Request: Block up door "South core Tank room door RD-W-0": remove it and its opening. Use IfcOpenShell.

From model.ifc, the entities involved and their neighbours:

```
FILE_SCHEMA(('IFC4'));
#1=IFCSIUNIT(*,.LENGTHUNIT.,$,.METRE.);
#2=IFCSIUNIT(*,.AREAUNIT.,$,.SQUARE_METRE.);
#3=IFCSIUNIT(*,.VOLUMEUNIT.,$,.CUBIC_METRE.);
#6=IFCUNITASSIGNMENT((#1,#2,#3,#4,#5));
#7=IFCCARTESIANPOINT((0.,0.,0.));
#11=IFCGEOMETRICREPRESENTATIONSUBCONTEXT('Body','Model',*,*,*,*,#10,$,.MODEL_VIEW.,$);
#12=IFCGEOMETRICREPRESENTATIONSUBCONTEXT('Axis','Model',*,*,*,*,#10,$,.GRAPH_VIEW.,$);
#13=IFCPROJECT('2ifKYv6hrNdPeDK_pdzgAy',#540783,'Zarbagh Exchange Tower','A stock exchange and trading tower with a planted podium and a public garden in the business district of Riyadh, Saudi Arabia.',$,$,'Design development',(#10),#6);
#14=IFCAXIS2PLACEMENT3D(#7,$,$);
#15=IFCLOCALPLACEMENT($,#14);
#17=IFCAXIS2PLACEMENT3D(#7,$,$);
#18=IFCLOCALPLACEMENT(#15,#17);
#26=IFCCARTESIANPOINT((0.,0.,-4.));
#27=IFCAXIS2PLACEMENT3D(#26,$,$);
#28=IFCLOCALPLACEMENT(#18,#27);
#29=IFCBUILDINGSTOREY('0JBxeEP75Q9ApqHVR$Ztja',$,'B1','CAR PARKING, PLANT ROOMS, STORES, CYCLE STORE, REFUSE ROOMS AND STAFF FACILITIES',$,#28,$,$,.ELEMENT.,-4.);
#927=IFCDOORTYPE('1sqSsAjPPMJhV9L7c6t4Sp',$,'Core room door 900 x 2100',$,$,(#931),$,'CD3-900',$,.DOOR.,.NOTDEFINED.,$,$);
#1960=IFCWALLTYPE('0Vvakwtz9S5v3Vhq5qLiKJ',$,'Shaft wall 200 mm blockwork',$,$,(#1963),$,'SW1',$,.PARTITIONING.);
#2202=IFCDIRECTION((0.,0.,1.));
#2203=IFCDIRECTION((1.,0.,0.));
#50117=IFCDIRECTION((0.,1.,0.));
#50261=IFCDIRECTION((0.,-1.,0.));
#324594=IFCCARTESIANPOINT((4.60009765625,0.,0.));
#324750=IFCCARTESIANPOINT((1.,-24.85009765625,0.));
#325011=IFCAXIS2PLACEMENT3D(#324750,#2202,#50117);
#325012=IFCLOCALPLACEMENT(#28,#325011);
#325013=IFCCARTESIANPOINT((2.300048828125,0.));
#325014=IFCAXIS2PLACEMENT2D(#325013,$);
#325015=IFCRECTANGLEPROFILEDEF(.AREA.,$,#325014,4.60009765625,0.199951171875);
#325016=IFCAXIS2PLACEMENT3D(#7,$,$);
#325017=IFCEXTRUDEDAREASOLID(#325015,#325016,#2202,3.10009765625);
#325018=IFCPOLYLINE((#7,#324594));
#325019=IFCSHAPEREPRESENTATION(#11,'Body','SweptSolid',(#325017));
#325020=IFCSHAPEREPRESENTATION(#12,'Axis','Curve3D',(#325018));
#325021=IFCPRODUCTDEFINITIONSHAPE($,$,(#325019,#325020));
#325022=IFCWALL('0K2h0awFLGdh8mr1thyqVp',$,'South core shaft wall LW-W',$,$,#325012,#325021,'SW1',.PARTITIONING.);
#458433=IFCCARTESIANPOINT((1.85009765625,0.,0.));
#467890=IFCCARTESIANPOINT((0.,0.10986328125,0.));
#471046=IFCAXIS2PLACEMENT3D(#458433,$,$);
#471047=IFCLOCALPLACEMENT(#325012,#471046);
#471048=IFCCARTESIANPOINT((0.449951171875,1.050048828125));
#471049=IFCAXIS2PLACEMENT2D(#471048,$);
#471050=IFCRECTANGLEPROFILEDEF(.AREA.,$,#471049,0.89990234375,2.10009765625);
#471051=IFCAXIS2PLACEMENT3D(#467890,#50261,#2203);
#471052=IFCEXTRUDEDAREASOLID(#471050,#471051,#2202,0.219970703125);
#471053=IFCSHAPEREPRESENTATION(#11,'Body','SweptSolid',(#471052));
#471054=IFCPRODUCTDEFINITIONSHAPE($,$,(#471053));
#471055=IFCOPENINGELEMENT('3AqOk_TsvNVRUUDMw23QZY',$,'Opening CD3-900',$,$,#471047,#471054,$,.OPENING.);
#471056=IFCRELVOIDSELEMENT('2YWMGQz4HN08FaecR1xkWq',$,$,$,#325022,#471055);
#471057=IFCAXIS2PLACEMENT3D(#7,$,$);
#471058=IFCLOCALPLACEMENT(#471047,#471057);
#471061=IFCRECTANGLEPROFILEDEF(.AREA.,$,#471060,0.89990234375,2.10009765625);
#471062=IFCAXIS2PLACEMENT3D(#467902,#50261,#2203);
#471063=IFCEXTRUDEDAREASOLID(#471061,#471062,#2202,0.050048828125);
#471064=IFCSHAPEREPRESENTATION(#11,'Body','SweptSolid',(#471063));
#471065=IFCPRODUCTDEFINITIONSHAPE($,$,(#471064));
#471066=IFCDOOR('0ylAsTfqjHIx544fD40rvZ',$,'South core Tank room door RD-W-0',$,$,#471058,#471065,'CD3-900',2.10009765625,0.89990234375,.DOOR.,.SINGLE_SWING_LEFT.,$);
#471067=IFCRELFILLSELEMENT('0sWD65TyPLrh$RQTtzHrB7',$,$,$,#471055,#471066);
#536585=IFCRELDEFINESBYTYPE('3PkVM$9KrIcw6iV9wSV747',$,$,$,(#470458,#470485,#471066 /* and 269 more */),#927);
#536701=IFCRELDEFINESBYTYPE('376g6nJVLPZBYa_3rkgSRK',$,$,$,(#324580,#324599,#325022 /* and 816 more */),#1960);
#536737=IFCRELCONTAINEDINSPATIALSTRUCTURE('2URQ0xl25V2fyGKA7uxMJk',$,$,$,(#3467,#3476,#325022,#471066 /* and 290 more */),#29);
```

```python
import ifcopenshell
import ifcopenshell.api.feature
import ifcopenshell.api.root
import ifcopenshell.geom
import ifcopenshell.util.shape

model = ifcopenshell.open("model.ifc")
settings = ifcopenshell.geom.settings()


def volume(element):
    """Net volume in cubic metres, openings subtracted."""
    shape = ifcopenshell.geom.create_shape(settings, element)
    return ifcopenshell.util.shape.get_volume(shape.geometry)


door = model.by_guid("0ylAsTfqjHIx544fD40rvZ")
opening = door.FillsVoids[0].RelatingOpeningElement
wall = opening.VoidsElements[0].RelatingBuildingElement
before = volume(wall)

ifcopenshell.api.root.remove_product(model, product=door)
ifcopenshell.api.feature.remove_feature(model, feature=opening)

after = volume(wall)

print(f"wall volume {before:.3f} -> {after:.3f} m3")

model.write("model_updated.ifc")
```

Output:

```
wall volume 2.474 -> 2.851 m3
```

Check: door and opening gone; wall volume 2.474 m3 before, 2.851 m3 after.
